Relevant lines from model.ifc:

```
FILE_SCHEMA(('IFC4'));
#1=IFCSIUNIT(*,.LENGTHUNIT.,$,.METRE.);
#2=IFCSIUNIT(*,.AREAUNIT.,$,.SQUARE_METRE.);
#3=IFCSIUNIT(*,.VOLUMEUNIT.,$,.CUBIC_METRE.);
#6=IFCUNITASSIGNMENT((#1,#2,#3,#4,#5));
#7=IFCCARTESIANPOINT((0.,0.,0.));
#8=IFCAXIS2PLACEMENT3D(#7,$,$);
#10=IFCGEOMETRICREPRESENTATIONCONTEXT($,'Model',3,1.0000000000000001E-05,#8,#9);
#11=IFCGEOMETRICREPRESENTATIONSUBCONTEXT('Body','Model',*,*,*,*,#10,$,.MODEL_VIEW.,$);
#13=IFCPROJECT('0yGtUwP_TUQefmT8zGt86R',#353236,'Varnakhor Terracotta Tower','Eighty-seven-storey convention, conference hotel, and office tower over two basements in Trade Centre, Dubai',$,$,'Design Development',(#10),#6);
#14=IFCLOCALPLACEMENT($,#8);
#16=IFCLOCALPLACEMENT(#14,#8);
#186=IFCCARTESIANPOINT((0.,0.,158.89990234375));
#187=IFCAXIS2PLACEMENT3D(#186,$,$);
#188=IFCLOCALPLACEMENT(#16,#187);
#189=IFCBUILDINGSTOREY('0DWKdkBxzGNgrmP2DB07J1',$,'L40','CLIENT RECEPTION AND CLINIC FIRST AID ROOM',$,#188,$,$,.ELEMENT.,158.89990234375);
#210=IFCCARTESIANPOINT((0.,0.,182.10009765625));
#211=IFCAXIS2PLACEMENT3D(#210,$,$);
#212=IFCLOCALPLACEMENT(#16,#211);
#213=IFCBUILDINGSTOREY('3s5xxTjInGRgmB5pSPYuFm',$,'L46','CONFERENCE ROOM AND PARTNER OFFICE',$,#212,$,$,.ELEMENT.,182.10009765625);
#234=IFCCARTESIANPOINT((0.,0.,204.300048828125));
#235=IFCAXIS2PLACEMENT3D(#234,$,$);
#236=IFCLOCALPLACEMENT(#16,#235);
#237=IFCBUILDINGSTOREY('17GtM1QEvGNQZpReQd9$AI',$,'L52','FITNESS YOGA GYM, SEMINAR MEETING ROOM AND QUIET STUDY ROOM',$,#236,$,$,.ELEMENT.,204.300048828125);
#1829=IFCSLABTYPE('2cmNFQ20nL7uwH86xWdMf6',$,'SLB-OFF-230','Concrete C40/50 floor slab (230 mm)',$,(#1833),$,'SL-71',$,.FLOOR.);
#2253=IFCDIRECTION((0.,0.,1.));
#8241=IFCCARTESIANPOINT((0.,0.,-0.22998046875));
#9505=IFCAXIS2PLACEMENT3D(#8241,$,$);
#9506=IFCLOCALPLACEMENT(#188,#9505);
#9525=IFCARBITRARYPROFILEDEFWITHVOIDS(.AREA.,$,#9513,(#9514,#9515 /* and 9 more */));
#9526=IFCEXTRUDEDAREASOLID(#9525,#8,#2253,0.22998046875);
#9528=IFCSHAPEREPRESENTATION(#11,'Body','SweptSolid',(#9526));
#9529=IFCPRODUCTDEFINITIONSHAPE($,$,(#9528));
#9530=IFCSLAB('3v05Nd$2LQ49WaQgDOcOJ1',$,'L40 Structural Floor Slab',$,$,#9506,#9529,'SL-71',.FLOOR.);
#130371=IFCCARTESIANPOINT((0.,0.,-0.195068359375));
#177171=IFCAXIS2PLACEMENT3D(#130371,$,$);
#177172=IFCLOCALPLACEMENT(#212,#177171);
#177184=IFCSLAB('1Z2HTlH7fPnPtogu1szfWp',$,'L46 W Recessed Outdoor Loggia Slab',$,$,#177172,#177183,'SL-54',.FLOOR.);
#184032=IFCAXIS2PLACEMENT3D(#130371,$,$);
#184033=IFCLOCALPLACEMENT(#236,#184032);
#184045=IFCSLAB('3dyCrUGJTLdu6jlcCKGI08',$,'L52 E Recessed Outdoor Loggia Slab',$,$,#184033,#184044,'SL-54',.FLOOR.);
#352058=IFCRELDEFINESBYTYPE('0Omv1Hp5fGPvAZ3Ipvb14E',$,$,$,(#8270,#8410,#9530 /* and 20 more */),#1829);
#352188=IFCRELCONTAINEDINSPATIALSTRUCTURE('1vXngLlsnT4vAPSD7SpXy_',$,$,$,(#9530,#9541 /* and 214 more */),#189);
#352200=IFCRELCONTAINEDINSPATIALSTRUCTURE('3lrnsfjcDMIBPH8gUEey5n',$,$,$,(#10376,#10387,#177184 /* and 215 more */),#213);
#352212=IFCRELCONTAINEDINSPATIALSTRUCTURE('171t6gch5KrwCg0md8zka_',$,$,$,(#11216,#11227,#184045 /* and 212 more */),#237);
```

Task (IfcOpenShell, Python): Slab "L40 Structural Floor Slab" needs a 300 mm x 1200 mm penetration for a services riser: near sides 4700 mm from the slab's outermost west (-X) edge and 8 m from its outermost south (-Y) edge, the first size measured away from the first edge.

```python
import numpy as np
import ifcopenshell
import ifcopenshell.api.feature
import ifcopenshell.api.geometry
import ifcopenshell.api.root
import ifcopenshell.geom
import ifcopenshell.util.placement
import ifcopenshell.util.representation
import ifcopenshell.util.shape
import ifcopenshell.util.unit

model = ifcopenshell.open("model.ifc")
unit_scale = ifcopenshell.util.unit.calculate_unit_scale(model)
settings = ifcopenshell.geom.settings()


def volume(element):
    """Net volume in cubic metres, openings subtracted."""
    shape = ifcopenshell.geom.create_shape(settings, element)
    return ifcopenshell.util.shape.get_volume(shape.geometry)


slab = model.by_guid("3v05Nd$2LQ49WaQgDOcOJ1")
before = volume(slab)

# Extent in the slab's own axes, in metres. The edges named are its -X and -Y sides.
slab_shape = ifcopenshell.geom.create_shape(settings, slab)
vertices = ifcopenshell.util.shape.get_vertices(slab_shape.geometry)
x_min, y_min, bottom = vertices.min(axis=0)
top = vertices[:, 2].max()

opening = ifcopenshell.api.root.create_entity(model, ifc_class="IfcOpeningElement", name="Services riser opening", predefined_type="OPENING")
context = ifcopenshell.util.representation.get_context(model, "Model", "Body", "MODEL_VIEW")
width, depth = 0.3, 1.2
outline = [(0.0, 0.0), (width, 0.0), (width, depth), (0.0, depth), (0.0, 0.0)]
# Overshoot both faces by 50 mm so the cut is clean.
shape = ifcopenshell.api.geometry.add_slab_representation(
    model, context=context, depth=top - bottom + 0.1, polyline=outline
)
ifcopenshell.api.geometry.assign_representation(model, product=opening, representation=shape)

matrix = ifcopenshell.util.placement.get_local_placement(slab.ObjectPlacement)
matrix[:, 3] = matrix @ np.append(np.array([x_min + 4.7, y_min + 8, bottom - 0.05]) / unit_scale, 1.0)
ifcopenshell.api.geometry.edit_object_placement(model, product=opening, matrix=matrix, is_si=False)
ifcopenshell.api.feature.add_feature(model, feature=opening, element=slab)

after = volume(slab)

print(f"slab volume {before:.3f} -> {after:.3f} m3")

model.write("model-out.ifc")
```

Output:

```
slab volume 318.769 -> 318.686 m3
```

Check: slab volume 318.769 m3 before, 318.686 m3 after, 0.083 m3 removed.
